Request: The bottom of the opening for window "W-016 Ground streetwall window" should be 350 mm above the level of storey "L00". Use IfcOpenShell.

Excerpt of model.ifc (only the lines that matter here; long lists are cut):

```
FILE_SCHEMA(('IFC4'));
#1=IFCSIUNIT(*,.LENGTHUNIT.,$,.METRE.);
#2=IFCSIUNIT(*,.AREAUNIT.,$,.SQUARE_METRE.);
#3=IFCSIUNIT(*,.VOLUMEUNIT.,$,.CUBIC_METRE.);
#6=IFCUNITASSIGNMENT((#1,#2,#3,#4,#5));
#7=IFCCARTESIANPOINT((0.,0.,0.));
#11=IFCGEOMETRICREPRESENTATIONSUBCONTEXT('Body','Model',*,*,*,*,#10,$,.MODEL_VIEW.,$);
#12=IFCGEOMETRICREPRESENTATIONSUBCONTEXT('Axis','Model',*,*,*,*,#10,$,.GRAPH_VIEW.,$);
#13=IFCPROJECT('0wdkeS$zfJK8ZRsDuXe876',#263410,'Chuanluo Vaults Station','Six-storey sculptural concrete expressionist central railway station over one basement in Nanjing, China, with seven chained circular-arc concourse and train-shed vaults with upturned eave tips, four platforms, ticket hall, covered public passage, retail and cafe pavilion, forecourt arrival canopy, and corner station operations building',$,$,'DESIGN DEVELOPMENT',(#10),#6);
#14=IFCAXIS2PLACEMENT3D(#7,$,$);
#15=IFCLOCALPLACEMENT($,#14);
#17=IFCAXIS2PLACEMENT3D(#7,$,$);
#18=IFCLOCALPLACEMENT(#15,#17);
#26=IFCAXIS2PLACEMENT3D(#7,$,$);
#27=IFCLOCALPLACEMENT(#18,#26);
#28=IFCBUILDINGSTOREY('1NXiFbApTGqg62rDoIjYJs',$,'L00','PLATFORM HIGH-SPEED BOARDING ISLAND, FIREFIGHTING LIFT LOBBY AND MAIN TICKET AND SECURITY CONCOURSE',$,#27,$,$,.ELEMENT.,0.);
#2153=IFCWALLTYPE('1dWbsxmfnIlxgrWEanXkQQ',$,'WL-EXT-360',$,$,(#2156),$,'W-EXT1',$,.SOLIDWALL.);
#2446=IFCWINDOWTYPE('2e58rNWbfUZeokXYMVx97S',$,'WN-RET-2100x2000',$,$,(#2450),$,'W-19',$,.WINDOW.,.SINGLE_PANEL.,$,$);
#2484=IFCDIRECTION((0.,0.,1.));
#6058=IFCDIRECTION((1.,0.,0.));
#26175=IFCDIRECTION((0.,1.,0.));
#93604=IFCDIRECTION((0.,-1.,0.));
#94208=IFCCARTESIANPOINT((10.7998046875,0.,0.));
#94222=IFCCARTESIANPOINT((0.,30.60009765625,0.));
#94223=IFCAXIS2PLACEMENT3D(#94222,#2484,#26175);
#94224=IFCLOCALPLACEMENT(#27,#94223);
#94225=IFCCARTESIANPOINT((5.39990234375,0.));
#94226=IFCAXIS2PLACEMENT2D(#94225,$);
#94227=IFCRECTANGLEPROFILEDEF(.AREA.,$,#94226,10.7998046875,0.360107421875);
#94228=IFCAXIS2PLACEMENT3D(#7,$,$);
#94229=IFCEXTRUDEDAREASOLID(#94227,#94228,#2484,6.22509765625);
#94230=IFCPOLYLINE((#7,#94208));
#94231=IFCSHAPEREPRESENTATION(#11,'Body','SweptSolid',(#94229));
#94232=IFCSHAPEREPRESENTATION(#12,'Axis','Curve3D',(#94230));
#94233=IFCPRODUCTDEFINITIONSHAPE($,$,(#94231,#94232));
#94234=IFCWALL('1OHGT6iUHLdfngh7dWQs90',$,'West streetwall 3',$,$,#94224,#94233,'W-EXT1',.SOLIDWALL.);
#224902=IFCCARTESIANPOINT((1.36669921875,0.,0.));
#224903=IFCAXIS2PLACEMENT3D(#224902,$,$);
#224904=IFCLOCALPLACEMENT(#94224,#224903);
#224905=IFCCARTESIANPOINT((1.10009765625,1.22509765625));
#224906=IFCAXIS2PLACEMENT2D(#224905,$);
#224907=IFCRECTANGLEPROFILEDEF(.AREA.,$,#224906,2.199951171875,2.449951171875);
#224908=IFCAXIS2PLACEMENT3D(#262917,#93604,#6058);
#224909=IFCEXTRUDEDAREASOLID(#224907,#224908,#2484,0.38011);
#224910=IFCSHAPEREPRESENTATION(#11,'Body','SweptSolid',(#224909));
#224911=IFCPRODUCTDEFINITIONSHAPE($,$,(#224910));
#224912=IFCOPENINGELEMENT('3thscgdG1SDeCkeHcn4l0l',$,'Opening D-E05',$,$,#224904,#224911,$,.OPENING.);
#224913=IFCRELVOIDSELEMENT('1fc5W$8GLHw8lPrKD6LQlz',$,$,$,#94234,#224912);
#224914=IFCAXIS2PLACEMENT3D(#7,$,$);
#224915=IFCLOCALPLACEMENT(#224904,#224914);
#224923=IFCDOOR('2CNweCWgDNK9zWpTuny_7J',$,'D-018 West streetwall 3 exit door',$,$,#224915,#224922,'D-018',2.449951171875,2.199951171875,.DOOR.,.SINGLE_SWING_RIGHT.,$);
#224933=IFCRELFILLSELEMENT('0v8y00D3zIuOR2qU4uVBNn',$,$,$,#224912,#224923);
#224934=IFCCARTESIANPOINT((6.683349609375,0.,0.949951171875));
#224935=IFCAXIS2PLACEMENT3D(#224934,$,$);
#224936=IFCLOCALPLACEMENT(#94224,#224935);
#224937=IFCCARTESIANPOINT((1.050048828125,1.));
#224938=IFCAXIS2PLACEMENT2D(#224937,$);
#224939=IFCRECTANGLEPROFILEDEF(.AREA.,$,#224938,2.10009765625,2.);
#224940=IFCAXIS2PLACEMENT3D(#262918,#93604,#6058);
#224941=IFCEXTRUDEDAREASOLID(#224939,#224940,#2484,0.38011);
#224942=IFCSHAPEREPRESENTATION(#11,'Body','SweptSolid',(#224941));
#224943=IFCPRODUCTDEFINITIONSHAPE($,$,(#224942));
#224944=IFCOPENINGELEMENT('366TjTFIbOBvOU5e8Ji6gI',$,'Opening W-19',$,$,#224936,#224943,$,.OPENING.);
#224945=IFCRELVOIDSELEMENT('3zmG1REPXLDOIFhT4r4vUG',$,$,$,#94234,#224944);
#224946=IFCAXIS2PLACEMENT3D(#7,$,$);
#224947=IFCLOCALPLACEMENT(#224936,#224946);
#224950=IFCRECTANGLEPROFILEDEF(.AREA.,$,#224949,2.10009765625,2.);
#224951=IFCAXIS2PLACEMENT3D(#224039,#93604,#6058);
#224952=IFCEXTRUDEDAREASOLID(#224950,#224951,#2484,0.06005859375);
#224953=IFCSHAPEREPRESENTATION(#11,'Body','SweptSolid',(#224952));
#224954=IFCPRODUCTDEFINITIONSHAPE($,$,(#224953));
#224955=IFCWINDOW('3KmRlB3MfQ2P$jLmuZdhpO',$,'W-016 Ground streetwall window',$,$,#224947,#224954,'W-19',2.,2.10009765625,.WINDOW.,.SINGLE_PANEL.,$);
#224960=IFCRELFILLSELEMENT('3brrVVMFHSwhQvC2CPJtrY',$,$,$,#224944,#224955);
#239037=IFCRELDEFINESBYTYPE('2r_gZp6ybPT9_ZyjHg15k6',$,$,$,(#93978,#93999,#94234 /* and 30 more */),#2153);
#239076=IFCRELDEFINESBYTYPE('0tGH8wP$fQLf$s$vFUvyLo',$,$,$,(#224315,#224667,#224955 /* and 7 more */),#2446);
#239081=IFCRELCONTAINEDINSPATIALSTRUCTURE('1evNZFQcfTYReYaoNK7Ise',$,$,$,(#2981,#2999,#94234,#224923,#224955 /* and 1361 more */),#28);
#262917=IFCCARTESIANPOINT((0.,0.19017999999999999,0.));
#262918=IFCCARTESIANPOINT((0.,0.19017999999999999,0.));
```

```python
import numpy as np
import ifcopenshell
import ifcopenshell.api.geometry
import ifcopenshell.geom
import ifcopenshell.util.element
import ifcopenshell.util.placement
import ifcopenshell.util.shape
import ifcopenshell.util.unit

model = ifcopenshell.open("model.ifc")
unit_scale = ifcopenshell.util.unit.calculate_unit_scale(model)

window = model.by_guid("3KmRlB3MfQ2P$jLmuZdhpO")
opening = window.FillsVoids[0].RelatingOpeningElement
storey = ifcopenshell.util.element.get_container(window, ifc_class="IfcBuildingStorey")
level = ifcopenshell.util.placement.get_local_placement(storey.ObjectPlacement)[2, 3]

# The opening's origin need not be at the sill, so measure its lowest point.
shape = ifcopenshell.geom.create_shape(ifcopenshell.geom.settings(), opening)
bottom = ifcopenshell.util.shape.get_shape_bottom_elevation(shape, shape.geometry) / unit_scale
dz = level + 0.35 / unit_scale - bottom

shift = np.array([0.0, 0.0, dz])
# The window is placed relative to its opening, so it follows when the opening moves.
matrix = ifcopenshell.util.placement.get_local_placement(opening.ObjectPlacement)
matrix[:3, 3] += shift
ifcopenshell.api.geometry.edit_object_placement(
    model, product=opening, matrix=matrix, is_si=False, should_transform_children=True
)

print(f"moved by {dz * unit_scale:+.3f} m")

model.write("model-out.ifc")
```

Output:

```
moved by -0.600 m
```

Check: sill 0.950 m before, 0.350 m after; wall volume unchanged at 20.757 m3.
